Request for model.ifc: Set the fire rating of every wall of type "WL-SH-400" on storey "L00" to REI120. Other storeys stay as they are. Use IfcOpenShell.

First a look at what the model holds.

```python
import ifcopenshell
import ifcopenshell.util.element

model = ifcopenshell.open("model.ifc")
print(model.schema)
storey = next(s for s in model.by_type("IfcBuildingStorey") if s.Name == "L00")
walls = [e for e in ifcopenshell.util.element.get_decomposition(storey) if e.is_a("IfcWall")]
seen = {}
for e in walls:
    element_type = ifcopenshell.util.element.get_type(e)
    key = (element_type.Name if element_type != e and element_type else None, ifcopenshell.util.element.get_pset(e, "Pset_WallCommon", "FireRating"))
    seen[key] = seen.get(key, 0) + 1
for (name, value), count in sorted(seen.items(), key=str):
    print(count, "x", name, "|", value)
```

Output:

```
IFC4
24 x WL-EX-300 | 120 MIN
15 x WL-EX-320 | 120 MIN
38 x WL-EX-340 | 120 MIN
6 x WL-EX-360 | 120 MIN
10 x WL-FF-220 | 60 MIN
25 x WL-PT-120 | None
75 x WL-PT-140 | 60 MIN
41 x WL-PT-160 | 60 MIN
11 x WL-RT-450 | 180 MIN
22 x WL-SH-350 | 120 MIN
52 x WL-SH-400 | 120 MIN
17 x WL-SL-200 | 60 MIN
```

```python
import ifcopenshell
import ifcopenshell.api.pset
import ifcopenshell.util.element

model = ifcopenshell.open("model.ifc")

storey = next(s for s in model.by_type("IfcBuildingStorey") if s.Name == "L00")
walls = [e for e in ifcopenshell.util.element.get_decomposition(storey) if e.is_a("IfcWall")]

count = 0
for e in walls:
    element_type = ifcopenshell.util.element.get_type(e)
    if element_type in (None, e) or element_type.Name != "WL-SH-400":
        continue
    # add_pset returns the element's existing set when there is one.
    pset = ifcopenshell.api.pset.add_pset(model, product=e, name="Pset_WallCommon")
    ifcopenshell.api.pset.edit_pset(model, pset=pset, properties={"FireRating": "REI120"})
    count += 1

print(count, "walls updated")

model.write("model_edited.ifc")
```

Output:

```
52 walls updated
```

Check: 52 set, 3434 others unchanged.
